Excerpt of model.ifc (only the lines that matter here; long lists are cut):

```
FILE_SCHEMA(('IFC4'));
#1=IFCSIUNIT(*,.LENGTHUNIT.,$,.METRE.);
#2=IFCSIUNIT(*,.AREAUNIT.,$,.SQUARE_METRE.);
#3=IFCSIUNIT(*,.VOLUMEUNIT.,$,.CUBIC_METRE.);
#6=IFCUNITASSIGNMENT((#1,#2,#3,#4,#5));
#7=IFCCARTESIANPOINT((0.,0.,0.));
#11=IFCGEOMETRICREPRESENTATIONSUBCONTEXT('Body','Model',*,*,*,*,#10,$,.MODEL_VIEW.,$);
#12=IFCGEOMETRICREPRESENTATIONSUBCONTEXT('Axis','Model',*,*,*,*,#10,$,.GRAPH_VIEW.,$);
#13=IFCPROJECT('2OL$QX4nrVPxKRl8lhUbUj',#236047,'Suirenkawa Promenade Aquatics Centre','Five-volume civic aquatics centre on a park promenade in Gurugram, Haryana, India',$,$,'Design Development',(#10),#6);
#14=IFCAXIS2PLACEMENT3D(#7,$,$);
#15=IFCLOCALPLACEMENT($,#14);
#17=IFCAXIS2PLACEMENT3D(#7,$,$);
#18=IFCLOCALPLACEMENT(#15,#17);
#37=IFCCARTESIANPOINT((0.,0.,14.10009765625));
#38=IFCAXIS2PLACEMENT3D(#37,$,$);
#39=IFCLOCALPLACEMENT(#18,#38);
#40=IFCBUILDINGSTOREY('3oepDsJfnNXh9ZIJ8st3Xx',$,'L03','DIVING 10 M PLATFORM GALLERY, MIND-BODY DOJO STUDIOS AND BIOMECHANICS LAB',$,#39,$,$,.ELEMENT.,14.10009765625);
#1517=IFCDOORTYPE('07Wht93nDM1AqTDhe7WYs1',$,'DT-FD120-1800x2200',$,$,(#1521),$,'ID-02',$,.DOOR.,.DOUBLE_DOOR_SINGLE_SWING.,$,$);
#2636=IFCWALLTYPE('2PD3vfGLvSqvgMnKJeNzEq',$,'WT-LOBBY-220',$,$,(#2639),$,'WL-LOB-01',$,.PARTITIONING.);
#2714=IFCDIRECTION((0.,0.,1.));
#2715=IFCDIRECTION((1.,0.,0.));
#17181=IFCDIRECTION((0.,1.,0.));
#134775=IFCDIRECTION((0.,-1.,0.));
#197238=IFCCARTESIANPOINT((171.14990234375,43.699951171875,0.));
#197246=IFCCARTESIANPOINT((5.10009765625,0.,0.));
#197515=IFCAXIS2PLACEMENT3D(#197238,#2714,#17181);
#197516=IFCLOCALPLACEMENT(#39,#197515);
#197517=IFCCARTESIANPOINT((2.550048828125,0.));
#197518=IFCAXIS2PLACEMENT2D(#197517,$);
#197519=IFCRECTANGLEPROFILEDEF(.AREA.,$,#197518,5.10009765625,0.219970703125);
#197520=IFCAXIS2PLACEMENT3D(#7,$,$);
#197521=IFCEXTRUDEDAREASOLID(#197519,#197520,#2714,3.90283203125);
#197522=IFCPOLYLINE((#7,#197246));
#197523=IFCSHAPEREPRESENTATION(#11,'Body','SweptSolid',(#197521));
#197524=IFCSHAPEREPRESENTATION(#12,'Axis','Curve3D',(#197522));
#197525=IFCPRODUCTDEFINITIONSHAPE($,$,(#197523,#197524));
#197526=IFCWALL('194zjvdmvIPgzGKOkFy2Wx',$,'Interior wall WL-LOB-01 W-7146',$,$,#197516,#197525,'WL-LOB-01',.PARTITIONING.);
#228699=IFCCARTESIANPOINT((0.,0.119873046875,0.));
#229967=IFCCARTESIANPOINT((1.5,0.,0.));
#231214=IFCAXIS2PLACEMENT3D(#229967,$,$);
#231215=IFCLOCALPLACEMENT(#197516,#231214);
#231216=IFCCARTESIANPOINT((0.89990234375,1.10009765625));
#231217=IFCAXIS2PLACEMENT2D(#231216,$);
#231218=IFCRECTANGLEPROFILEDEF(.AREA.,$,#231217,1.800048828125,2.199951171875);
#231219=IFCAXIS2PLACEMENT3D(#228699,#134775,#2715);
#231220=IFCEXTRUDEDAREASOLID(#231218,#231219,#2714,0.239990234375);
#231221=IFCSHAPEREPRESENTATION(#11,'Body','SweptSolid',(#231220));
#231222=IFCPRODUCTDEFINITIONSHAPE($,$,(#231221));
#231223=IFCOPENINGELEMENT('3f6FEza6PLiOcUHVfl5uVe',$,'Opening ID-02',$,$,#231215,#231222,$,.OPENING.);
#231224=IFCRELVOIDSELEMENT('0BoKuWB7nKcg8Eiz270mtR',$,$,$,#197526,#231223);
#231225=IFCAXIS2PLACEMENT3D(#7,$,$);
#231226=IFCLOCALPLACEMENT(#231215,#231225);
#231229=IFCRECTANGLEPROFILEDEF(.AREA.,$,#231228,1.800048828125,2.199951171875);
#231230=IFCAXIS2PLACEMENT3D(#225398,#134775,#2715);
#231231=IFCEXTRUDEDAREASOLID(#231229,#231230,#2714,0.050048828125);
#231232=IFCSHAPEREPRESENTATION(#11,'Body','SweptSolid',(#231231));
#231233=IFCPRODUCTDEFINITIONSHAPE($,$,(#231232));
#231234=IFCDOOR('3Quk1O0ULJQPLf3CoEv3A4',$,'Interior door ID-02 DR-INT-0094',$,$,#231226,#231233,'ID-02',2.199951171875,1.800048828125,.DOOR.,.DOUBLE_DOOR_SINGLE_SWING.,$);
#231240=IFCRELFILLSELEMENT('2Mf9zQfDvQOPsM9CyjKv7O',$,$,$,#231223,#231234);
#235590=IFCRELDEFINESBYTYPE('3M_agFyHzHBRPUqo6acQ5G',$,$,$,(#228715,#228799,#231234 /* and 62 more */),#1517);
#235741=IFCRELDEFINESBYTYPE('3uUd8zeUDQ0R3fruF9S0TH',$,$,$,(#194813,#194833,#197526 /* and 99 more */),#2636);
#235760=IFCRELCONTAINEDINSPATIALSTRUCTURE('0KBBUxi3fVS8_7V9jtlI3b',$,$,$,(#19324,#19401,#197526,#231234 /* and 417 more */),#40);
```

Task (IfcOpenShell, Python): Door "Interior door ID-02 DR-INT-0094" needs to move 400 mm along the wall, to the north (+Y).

```python
import ifcopenshell
import ifcopenshell.api.geometry
import ifcopenshell.util.placement
import ifcopenshell.util.unit

model = ifcopenshell.open("model.ifc")
unit_scale = ifcopenshell.util.unit.calculate_unit_scale(model)

door = model.by_guid("3Quk1O0ULJQPLf3CoEv3A4")
opening = door.FillsVoids[0].RelatingOpeningElement
wall = opening.VoidsElements[0].RelatingBuildingElement

wall_matrix = ifcopenshell.util.placement.get_local_placement(wall.ObjectPlacement)
shift = wall_matrix[:3, 0] * 0.4 / unit_scale
before = ifcopenshell.util.placement.get_local_placement(door.ObjectPlacement)[:3, 3].copy()

# The door is placed relative to its opening, so it follows when the opening moves.
matrix = ifcopenshell.util.placement.get_local_placement(opening.ObjectPlacement)
matrix[:3, 3] += shift
ifcopenshell.api.geometry.edit_object_placement(
    model, product=opening, matrix=matrix, is_si=False, should_transform_children=True
)

after = ifcopenshell.util.placement.get_local_placement(door.ObjectPlacement)[:3, 3]
print("door moved by", (after - before).round(3) + 0.0)

model.write("model-out.ifc")
```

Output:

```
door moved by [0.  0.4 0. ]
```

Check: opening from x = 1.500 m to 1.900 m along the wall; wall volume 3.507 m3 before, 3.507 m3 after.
